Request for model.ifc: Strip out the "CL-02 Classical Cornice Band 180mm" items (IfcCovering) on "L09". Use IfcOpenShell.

First a look at what the model holds.

```python
import ifcopenshell
import ifcopenshell.util.element

model = ifcopenshell.open("model.ifc")
print(model.schema)
storey = next(s for s in model.by_type("IfcBuildingStorey") if s.Name == "L09")
coverings = [e for e in ifcopenshell.util.element.get_decomposition(storey) if e.is_a("IfcCovering")]
seen = {}
for e in coverings:
    element_type = ifcopenshell.util.element.get_type(e)
    name = element_type.Name if element_type not in (None, e) else None
    seen[name] = seen.get(name, 0) + 1
for name, count in sorted(seen.items(), key=str):
    print(count, "x", name)
```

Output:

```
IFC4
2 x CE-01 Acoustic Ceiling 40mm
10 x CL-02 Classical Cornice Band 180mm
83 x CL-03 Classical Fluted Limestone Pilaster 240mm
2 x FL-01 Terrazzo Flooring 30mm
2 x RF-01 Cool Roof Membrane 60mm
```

```python
import ifcopenshell
import ifcopenshell.api.root
import ifcopenshell.util.element

model = ifcopenshell.open("model.ifc")

storey = next(s for s in model.by_type("IfcBuildingStorey") if s.Name == "L09")
coverings = [e for e in ifcopenshell.util.element.get_decomposition(storey) if e.is_a("IfcCovering")]
targets = [e for e in coverings if (t := ifcopenshell.util.element.get_type(e)) not in (None, e) and t.Name == "CL-02 Classical Cornice Band 180mm"]

for e in targets:
    ifcopenshell.api.root.remove_product(model, product=e)
print(len(targets), "removed")

model.write("model_updated.ifc")
```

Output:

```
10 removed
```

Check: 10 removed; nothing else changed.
